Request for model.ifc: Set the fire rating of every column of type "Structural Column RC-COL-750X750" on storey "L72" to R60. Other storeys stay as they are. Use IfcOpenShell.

First a look at what the model holds.

```python
import ifcopenshell
import ifcopenshell.util.element

model = ifcopenshell.open("model.ifc")
print(model.schema)
storey = next(s for s in model.by_type("IfcBuildingStorey") if s.Name == "L72")
columns = [e for e in ifcopenshell.util.element.get_decomposition(storey) if e.is_a("IfcColumn")]
seen = {}
for e in columns:
    element_type = ifcopenshell.util.element.get_type(e)
    key = (element_type.Name if element_type != e and element_type else None, ifcopenshell.util.element.get_pset(e, "Pset_ColumnCommon", "FireRating"))
    seen[key] = seen.get(key, 0) + 1
for (name, value), count in sorted(seen.items(), key=str):
    print(count, "x", name, "|", value)
```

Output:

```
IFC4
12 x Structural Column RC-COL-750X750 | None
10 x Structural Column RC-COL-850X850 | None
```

```python
import ifcopenshell
import ifcopenshell.api.pset
import ifcopenshell.util.element

model = ifcopenshell.open("model.ifc")

storey = next(s for s in model.by_type("IfcBuildingStorey") if s.Name == "L72")
columns = [e for e in ifcopenshell.util.element.get_decomposition(storey) if e.is_a("IfcColumn")]

count = 0
for e in columns:
    element_type = ifcopenshell.util.element.get_type(e)
    if element_type in (None, e) or element_type.Name != "Structural Column RC-COL-750X750":
        continue
    found = ifcopenshell.util.element.get_pset(e, "Pset_ColumnCommon", should_inherit=False)
    if found:
        pset = model.by_id(found["id"])
        if len(ifcopenshell.util.element.get_elements_by_pset(pset)) > 1:
            pset = ifcopenshell.api.pset.unshare_pset(model, products=[e], pset=pset)[0]
    else:
        pset = ifcopenshell.api.pset.add_pset(model, product=e, name="Pset_ColumnCommon")
    ifcopenshell.api.pset.edit_pset(model, pset=pset, properties={"FireRating": "R60"})
    count += 1

print(count, "columns updated")

model.write("model_v2.ifc")
```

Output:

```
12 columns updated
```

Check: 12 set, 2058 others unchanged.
